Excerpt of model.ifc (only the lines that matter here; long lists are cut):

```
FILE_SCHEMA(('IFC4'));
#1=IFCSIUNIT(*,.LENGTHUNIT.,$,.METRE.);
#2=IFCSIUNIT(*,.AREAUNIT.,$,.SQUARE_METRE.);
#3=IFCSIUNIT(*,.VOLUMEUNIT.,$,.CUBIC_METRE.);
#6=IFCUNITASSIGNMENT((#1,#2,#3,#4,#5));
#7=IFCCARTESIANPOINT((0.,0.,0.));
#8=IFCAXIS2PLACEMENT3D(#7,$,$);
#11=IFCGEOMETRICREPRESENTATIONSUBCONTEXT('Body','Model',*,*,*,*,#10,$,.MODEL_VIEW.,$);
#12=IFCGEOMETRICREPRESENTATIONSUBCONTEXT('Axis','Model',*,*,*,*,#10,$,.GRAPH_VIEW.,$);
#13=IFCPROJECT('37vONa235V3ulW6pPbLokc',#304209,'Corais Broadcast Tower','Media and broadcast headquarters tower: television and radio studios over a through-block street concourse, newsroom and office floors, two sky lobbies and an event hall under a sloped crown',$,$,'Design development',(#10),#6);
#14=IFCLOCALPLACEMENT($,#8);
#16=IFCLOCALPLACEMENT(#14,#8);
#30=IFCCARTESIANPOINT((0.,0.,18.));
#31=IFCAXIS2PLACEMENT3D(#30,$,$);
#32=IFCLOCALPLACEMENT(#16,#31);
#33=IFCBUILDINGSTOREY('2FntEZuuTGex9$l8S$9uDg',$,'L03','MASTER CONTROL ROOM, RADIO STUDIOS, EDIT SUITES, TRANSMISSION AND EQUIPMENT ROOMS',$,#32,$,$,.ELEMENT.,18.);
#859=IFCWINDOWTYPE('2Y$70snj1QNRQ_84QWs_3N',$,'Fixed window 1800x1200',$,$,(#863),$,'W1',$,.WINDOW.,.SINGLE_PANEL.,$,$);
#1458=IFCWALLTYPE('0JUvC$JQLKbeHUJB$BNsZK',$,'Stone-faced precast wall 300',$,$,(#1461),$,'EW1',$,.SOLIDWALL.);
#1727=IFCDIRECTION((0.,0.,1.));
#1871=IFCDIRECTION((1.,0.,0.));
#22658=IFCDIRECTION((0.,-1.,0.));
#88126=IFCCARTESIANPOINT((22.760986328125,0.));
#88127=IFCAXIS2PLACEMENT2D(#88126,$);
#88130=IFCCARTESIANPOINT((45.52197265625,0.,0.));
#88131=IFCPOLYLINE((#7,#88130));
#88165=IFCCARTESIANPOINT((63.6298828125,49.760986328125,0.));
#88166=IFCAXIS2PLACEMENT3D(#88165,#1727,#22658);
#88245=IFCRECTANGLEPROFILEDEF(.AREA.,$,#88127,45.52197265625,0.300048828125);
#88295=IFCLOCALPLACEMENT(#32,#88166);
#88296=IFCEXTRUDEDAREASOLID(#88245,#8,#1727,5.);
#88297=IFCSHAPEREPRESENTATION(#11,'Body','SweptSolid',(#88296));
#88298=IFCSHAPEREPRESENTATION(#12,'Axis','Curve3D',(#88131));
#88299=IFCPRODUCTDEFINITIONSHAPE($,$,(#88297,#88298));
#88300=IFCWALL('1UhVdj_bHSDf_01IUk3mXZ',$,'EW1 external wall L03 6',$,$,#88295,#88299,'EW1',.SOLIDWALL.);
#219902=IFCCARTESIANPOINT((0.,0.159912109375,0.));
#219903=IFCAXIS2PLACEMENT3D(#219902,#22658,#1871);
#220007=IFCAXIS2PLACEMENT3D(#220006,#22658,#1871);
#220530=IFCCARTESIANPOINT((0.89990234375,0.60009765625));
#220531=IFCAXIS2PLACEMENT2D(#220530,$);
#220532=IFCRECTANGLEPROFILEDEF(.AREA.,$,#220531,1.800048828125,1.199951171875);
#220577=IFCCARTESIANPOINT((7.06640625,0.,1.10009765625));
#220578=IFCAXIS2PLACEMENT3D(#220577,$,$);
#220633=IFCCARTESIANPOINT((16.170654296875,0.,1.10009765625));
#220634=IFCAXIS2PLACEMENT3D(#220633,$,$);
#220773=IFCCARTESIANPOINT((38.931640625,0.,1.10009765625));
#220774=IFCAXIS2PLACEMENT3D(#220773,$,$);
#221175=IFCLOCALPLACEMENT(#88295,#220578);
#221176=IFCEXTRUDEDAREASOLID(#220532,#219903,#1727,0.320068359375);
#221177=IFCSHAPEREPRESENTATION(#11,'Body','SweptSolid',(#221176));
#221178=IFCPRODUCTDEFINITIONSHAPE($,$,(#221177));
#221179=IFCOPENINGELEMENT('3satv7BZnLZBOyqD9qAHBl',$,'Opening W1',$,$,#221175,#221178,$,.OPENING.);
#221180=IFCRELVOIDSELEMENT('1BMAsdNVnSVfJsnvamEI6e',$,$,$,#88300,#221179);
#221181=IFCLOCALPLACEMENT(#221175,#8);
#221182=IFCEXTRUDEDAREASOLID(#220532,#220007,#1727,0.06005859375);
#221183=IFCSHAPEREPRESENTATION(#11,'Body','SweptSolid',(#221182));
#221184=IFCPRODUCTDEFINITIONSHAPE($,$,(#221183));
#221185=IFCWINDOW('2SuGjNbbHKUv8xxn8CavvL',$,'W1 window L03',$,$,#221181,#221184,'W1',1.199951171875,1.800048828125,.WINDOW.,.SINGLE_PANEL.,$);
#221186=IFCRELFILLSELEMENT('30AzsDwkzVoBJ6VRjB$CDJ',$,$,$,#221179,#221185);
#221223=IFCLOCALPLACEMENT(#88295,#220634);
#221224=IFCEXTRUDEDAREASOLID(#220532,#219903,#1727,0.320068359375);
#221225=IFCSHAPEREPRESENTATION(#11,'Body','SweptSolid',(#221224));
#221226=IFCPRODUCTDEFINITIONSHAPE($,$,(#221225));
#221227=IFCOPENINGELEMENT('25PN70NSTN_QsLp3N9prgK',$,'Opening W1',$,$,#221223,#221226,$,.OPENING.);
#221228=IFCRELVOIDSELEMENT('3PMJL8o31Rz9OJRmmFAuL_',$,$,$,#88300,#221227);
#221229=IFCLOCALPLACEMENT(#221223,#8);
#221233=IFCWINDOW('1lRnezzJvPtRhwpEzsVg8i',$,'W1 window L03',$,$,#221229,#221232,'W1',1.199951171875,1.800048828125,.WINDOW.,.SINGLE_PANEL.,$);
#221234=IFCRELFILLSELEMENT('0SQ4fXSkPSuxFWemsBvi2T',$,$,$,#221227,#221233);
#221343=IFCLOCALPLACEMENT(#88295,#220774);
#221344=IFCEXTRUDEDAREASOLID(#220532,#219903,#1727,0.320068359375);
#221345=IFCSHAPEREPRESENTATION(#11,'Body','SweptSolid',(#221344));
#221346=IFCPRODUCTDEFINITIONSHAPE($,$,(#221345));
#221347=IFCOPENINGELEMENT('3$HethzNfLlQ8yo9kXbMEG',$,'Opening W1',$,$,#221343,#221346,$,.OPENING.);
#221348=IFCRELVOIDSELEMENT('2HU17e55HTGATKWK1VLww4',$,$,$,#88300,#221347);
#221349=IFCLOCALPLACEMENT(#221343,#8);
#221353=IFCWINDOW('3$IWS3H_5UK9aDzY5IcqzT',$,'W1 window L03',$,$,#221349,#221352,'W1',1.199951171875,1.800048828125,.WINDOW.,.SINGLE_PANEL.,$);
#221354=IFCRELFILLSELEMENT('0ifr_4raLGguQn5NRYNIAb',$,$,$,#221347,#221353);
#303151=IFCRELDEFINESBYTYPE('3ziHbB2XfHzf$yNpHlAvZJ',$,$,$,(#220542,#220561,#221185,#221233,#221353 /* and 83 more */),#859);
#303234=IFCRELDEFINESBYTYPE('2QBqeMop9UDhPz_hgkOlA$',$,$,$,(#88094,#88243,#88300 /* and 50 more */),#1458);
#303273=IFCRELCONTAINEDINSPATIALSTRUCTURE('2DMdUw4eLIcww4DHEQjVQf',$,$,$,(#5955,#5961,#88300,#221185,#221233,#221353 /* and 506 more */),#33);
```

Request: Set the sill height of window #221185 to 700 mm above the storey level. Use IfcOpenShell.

```python
import numpy as np
import ifcopenshell
import ifcopenshell.api.geometry
import ifcopenshell.geom
import ifcopenshell.util.element
import ifcopenshell.util.placement
import ifcopenshell.util.shape
import ifcopenshell.util.unit

model = ifcopenshell.open("model.ifc")
unit_scale = ifcopenshell.util.unit.calculate_unit_scale(model)

window = model.by_guid("2SuGjNbbHKUv8xxn8CavvL")
opening = window.FillsVoids[0].RelatingOpeningElement
storey = ifcopenshell.util.element.get_container(window, ifc_class="IfcBuildingStorey")
level = ifcopenshell.util.placement.get_local_placement(storey.ObjectPlacement)[2, 3]

# The opening's origin need not be at the sill, so measure its lowest point.
shape = ifcopenshell.geom.create_shape(ifcopenshell.geom.settings(), opening)
bottom = ifcopenshell.util.shape.get_shape_bottom_elevation(shape, shape.geometry) / unit_scale
dz = level + 0.7 - bottom

shift = np.array([0.0, 0.0, dz])
# The window is placed relative to its opening, so it follows when the opening moves.
matrix = ifcopenshell.util.placement.get_local_placement(opening.ObjectPlacement)
matrix[:3, 3] += shift
ifcopenshell.api.geometry.edit_object_placement(
    model, product=opening, matrix=matrix, is_si=False, should_transform_children=True
)

print(f"moved by {dz * unit_scale:+.3f} m")

model.write("model_rev.ifc")
```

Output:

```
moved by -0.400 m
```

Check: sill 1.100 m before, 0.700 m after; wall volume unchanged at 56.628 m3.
